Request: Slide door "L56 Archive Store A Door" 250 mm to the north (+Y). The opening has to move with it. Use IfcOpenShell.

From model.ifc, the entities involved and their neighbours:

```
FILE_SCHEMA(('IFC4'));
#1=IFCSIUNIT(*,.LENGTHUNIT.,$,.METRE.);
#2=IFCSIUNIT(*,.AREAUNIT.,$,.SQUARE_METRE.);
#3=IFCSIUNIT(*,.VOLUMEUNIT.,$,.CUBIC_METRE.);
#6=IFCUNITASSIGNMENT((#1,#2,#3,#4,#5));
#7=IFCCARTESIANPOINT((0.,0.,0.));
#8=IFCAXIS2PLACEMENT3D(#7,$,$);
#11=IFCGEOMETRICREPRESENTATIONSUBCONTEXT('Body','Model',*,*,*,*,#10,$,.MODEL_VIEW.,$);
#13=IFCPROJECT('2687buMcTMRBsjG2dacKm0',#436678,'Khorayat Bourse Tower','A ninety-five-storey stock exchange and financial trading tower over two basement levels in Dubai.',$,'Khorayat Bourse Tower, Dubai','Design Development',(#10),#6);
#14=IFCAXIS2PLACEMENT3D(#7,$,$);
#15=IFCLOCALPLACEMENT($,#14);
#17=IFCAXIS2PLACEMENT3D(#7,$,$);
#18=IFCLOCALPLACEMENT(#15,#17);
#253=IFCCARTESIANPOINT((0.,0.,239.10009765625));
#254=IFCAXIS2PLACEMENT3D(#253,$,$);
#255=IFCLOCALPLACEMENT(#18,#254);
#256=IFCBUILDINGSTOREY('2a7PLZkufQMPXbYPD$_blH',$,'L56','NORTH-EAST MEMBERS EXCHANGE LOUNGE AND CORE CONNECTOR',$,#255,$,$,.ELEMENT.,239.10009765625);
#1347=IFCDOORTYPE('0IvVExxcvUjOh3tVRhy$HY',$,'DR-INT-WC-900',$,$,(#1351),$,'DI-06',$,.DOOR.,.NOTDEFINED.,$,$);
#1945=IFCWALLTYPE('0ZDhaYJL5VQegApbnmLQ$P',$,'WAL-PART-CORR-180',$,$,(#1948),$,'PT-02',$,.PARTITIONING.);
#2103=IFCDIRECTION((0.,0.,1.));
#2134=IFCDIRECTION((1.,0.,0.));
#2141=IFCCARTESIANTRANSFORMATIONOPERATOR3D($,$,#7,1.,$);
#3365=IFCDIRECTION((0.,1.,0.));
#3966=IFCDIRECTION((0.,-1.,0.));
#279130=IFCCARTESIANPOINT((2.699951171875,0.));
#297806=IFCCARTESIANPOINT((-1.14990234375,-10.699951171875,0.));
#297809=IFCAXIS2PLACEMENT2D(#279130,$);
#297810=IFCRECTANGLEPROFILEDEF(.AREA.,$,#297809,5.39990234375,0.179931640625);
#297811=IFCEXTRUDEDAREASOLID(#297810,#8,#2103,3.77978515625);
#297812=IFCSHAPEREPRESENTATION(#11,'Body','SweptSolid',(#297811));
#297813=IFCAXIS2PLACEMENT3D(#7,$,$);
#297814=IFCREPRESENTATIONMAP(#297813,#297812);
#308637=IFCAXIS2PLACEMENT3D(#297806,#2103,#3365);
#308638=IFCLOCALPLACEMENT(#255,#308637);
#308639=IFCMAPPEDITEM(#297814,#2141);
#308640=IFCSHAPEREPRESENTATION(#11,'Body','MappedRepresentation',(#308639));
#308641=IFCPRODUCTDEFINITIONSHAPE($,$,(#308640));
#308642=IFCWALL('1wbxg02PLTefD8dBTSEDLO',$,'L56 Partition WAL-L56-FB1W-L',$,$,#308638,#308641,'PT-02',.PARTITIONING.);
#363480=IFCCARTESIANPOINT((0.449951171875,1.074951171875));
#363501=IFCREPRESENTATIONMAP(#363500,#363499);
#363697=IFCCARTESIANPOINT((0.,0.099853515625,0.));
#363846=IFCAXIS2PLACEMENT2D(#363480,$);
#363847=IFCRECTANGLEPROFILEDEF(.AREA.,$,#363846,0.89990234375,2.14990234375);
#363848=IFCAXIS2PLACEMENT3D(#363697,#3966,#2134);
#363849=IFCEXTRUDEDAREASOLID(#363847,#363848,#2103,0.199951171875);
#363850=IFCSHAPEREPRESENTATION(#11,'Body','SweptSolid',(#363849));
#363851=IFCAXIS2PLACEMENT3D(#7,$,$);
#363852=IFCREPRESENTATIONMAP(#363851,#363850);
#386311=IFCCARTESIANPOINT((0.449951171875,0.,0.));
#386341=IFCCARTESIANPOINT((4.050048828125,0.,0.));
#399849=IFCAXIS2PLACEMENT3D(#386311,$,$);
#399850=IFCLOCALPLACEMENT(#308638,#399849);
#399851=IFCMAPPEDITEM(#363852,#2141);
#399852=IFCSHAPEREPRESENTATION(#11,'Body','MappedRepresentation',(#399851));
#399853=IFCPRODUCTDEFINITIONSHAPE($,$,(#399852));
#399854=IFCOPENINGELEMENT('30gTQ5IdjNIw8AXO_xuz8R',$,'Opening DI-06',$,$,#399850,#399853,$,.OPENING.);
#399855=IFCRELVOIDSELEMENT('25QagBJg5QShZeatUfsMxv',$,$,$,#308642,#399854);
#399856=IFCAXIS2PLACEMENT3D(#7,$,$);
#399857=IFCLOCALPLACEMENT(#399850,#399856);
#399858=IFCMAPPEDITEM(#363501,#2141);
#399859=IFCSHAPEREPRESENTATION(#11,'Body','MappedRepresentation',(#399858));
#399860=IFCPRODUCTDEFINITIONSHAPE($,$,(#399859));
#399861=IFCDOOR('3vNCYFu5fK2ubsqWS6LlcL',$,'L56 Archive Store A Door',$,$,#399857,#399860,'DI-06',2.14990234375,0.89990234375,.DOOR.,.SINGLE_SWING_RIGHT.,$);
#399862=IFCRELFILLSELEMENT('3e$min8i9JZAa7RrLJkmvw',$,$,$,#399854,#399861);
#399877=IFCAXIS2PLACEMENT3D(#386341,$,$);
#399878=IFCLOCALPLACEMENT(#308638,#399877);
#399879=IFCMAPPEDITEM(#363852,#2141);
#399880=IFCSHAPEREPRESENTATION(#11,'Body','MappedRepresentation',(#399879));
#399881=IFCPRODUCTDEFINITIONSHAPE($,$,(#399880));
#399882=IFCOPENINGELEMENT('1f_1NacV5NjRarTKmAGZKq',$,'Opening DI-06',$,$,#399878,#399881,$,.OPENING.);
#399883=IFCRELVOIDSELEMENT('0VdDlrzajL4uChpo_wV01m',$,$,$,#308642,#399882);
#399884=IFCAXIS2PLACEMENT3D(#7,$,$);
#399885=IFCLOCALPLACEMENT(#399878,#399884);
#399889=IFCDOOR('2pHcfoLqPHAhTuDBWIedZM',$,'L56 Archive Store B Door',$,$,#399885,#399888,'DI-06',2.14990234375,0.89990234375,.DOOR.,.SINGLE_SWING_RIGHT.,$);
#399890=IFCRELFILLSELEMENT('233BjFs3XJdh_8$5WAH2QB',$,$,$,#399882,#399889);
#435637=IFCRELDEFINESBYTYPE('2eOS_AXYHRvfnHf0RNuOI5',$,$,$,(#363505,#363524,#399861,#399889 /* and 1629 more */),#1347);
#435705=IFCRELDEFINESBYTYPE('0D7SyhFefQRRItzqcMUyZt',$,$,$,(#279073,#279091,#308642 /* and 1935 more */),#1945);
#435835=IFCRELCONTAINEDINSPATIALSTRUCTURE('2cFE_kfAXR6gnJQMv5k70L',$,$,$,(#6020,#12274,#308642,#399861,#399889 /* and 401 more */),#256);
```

```python
import ifcopenshell
import ifcopenshell.api.geometry
import ifcopenshell.util.placement

model = ifcopenshell.open("model.ifc")

door = model.by_guid("3vNCYFu5fK2ubsqWS6LlcL")
opening = door.FillsVoids[0].RelatingOpeningElement
wall = opening.VoidsElements[0].RelatingBuildingElement

wall_matrix = ifcopenshell.util.placement.get_local_placement(wall.ObjectPlacement)
shift = wall_matrix[:3, 0] * 0.25
before = ifcopenshell.util.placement.get_local_placement(door.ObjectPlacement)[:3, 3].copy()

# The door is placed relative to its opening, so it follows when the opening moves.
matrix = ifcopenshell.util.placement.get_local_placement(opening.ObjectPlacement)
matrix[:3, 3] += shift
ifcopenshell.api.geometry.edit_object_placement(
    model, product=opening, matrix=matrix, is_si=False, should_transform_children=True
)

after = ifcopenshell.util.placement.get_local_placement(door.ObjectPlacement)[:3, 3]
print("door moved by", (after - before).round(3) + 0.0)

model.write("model_updated.ifc")
```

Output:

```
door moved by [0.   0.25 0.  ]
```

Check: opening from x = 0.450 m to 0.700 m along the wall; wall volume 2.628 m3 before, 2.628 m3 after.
